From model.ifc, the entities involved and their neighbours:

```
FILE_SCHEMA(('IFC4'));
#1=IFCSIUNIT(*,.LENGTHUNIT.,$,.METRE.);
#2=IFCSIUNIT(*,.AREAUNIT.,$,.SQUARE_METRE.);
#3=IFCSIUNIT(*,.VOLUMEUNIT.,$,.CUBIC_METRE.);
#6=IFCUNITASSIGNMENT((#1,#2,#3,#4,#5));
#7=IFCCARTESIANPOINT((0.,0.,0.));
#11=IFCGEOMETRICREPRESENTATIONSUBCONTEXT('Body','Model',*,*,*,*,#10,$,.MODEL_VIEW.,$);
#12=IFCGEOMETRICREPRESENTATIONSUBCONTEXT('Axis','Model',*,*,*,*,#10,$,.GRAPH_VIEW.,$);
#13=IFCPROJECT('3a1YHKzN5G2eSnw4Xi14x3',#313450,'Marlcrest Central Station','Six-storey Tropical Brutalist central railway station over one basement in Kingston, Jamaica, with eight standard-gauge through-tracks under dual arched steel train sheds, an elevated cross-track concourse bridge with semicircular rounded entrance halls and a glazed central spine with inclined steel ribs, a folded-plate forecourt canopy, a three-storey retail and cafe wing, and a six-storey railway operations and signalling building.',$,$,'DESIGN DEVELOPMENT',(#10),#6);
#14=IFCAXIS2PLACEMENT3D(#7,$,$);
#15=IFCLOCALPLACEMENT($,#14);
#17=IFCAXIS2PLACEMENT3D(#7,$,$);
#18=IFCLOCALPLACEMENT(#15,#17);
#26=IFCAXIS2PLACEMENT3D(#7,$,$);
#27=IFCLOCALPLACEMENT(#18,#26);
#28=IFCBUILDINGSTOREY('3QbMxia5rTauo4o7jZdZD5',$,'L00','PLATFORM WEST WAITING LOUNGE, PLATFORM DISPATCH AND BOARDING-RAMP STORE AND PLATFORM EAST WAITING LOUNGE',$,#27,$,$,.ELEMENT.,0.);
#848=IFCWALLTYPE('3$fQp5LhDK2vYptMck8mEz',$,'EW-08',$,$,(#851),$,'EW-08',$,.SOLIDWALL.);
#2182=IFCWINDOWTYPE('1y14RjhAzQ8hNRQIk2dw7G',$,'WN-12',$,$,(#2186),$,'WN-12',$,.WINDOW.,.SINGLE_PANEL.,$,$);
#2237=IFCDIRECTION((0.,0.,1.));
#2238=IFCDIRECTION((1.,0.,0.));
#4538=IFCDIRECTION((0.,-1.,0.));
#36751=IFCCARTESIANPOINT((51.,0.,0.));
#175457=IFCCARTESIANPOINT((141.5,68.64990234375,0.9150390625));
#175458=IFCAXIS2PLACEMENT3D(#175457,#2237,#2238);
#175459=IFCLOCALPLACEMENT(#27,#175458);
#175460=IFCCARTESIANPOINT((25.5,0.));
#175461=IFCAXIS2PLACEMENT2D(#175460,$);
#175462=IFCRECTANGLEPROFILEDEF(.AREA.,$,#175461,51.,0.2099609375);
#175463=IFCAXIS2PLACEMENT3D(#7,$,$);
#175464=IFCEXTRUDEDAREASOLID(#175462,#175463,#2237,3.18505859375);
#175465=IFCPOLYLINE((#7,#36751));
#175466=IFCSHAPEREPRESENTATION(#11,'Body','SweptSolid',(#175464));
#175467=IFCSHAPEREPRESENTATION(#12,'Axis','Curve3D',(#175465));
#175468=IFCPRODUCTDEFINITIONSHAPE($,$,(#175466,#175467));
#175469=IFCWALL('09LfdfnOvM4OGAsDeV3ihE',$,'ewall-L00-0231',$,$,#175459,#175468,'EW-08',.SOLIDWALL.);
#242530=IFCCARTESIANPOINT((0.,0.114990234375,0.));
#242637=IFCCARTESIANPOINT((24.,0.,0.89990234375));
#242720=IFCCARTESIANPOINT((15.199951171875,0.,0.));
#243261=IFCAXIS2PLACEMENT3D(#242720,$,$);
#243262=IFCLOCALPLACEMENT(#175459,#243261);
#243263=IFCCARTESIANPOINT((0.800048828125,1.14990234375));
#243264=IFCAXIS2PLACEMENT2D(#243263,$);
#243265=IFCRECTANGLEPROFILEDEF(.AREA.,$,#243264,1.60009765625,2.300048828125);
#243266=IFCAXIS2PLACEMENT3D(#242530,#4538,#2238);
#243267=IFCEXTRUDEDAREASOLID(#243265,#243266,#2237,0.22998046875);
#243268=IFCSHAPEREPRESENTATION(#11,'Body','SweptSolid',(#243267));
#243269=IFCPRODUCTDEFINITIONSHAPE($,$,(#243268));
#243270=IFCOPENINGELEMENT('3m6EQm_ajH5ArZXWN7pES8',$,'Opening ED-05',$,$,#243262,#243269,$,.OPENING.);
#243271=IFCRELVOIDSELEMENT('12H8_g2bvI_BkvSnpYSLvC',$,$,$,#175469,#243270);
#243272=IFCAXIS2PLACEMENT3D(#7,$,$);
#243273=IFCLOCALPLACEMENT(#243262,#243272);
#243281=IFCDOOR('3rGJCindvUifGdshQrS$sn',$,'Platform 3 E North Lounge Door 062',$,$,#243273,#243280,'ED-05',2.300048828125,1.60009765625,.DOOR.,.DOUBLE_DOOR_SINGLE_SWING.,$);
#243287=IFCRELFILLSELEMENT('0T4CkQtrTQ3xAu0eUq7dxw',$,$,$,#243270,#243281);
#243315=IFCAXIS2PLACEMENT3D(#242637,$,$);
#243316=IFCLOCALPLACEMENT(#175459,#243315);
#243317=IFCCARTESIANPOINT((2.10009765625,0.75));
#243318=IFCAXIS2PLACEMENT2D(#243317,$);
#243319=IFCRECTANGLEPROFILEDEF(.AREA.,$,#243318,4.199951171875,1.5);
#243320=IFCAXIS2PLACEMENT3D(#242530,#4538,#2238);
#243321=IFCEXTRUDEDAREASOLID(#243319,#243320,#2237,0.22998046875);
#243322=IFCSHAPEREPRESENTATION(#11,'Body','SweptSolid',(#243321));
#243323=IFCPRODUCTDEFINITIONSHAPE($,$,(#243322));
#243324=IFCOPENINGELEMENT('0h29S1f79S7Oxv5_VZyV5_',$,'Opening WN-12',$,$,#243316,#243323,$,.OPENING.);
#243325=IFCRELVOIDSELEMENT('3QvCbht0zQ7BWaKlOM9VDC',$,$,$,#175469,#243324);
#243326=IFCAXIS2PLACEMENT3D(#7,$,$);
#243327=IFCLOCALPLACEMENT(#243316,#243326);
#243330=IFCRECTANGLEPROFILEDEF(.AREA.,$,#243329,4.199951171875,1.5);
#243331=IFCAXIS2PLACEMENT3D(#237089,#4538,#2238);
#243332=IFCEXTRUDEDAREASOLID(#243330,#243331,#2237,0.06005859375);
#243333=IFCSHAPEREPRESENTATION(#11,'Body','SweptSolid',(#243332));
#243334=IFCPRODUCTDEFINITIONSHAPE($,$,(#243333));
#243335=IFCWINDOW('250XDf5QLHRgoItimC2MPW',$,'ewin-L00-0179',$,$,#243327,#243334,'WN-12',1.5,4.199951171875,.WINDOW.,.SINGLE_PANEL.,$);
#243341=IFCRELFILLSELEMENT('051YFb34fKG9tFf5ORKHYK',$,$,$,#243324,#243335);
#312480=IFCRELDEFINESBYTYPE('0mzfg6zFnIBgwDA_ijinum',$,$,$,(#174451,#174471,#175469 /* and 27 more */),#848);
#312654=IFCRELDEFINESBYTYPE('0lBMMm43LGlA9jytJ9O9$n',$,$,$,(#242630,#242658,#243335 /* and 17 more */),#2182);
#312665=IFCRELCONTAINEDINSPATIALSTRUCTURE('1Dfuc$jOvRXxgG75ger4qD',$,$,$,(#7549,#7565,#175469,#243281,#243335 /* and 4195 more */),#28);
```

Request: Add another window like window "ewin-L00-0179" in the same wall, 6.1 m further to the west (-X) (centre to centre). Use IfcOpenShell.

```python
import ifcopenshell
import ifcopenshell.api.feature
import ifcopenshell.api.geometry
import ifcopenshell.api.root
import ifcopenshell.geom
import ifcopenshell.util.element
import ifcopenshell.util.placement
import ifcopenshell.util.shape

model = ifcopenshell.open("model.ifc")
settings = ifcopenshell.geom.settings()


def volume(element):
    """Net volume in cubic metres, openings subtracted."""
    shape = ifcopenshell.geom.create_shape(settings, element)
    return ifcopenshell.util.shape.get_volume(shape.geometry)


window = model.by_id(243335)
opening = window.FillsVoids[0].RelatingOpeningElement
wall = opening.VoidsElements[0].RelatingBuildingElement
before = volume(wall)
shift = ifcopenshell.util.placement.get_local_placement(wall.ObjectPlacement)[:3, 0] * -6.1

# copy_class copies the void relationship, type, container and properties, but no geometry.
new_opening = ifcopenshell.api.root.copy_class(model, product=opening)
new_opening.Representation = ifcopenshell.util.element.copy_deep(
    model, opening.Representation, exclude=["IfcGeometricRepresentationContext", "IfcRepresentationMap"]
)
new_window = ifcopenshell.api.root.copy_class(model, product=window)
new_window.Representation = ifcopenshell.util.element.copy_deep(
    model, window.Representation, exclude=["IfcGeometricRepresentationContext", "IfcRepresentationMap"]
)
new_window.Tag = None
ifcopenshell.api.feature.add_filling(model, opening=new_opening, element=new_window)

for old, new in ((opening, new_opening), (window, new_window)):
    matrix = ifcopenshell.util.placement.get_local_placement(old.ObjectPlacement)
    matrix[:3, 3] += shift
    ifcopenshell.api.geometry.edit_object_placement(model, product=new, matrix=matrix, is_si=False)

after = volume(wall)

print(f"wall volume {before:.3f} -> {after:.3f} m3")

model.write("model_rev.ifc")
```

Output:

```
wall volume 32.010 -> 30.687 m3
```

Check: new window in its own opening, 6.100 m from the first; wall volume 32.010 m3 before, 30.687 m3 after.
